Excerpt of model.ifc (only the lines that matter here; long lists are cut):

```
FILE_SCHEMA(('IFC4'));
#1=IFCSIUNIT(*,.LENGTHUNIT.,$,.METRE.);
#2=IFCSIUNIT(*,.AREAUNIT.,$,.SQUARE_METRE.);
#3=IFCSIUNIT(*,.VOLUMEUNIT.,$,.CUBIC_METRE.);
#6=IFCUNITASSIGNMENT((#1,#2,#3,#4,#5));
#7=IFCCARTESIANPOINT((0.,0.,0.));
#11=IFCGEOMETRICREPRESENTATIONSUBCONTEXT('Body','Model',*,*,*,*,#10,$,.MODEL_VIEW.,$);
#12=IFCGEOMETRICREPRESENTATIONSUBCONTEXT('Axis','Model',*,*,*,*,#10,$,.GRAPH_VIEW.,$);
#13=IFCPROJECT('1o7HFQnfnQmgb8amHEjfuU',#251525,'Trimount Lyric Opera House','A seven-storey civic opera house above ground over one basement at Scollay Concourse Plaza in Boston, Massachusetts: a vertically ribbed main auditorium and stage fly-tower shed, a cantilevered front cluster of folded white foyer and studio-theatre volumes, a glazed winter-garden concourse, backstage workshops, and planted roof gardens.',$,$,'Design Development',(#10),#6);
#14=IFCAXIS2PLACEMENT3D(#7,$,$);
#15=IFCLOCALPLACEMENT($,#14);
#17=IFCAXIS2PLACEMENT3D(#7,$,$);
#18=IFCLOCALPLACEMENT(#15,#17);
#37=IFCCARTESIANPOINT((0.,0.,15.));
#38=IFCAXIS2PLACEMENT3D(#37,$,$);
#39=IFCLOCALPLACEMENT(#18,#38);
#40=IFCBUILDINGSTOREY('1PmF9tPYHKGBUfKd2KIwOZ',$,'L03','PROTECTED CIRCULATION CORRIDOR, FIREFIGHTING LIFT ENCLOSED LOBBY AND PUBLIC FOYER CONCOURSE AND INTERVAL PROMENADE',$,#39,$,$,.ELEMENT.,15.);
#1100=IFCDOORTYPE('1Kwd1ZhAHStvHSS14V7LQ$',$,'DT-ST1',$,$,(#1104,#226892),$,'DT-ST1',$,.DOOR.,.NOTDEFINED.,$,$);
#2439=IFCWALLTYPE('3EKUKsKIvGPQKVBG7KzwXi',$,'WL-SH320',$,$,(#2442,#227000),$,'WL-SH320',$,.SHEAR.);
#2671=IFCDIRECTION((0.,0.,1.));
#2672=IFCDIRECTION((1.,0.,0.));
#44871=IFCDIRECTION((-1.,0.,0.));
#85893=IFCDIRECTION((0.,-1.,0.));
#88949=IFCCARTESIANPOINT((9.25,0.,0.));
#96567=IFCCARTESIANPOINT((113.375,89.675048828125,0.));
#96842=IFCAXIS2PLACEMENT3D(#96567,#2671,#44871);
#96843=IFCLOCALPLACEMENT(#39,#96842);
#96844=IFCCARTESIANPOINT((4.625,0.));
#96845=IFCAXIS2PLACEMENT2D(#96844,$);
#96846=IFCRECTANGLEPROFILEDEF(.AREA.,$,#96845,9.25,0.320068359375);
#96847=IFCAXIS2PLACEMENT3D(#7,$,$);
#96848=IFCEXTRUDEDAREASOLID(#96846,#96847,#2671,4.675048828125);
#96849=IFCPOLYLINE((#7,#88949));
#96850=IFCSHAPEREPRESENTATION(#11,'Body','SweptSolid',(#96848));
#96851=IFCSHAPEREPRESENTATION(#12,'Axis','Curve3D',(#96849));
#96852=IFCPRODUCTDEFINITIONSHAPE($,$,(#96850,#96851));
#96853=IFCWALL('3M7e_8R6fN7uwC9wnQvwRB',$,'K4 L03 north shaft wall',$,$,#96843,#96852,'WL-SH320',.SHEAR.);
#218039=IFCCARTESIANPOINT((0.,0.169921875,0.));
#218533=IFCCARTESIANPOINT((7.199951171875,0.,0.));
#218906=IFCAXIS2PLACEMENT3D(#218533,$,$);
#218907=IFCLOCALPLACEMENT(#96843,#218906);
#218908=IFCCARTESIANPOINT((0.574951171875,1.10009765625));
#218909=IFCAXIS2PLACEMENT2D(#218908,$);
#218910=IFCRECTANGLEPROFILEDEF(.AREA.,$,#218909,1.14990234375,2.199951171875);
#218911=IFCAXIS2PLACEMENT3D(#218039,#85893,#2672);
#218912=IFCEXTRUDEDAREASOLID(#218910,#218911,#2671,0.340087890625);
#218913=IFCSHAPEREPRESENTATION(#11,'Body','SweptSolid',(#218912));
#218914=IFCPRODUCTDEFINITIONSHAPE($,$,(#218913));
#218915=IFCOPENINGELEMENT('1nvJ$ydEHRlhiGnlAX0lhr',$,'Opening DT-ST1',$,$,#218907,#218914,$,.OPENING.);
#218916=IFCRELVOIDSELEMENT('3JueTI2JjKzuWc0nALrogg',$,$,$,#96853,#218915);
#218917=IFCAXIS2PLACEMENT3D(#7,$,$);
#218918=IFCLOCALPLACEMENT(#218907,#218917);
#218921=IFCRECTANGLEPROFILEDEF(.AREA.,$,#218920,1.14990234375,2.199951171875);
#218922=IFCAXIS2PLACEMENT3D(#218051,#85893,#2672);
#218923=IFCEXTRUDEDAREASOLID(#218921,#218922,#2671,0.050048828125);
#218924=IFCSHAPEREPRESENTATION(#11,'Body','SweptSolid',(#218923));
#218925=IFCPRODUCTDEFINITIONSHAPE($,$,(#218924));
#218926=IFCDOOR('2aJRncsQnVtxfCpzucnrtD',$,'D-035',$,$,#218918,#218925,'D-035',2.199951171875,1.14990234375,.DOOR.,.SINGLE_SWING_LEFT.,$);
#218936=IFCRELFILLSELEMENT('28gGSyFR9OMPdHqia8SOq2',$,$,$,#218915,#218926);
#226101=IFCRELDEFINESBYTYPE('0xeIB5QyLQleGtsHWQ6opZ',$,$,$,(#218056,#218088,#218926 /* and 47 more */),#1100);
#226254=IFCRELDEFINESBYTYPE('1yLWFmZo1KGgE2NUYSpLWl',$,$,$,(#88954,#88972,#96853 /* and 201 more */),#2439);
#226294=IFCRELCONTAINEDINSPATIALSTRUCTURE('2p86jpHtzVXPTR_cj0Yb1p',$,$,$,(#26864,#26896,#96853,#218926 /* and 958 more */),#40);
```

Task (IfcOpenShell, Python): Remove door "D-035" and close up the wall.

```python
import ifcopenshell
import ifcopenshell.api.feature
import ifcopenshell.api.root
import ifcopenshell.geom
import ifcopenshell.util.shape

model = ifcopenshell.open("model.ifc")
settings = ifcopenshell.geom.settings()


def volume(element):
    """Net volume in cubic metres, openings subtracted."""
    shape = ifcopenshell.geom.create_shape(settings, element)
    return ifcopenshell.util.shape.get_volume(shape.geometry)


door = model.by_guid("2aJRncsQnVtxfCpzucnrtD")
opening = door.FillsVoids[0].RelatingOpeningElement
wall = opening.VoidsElements[0].RelatingBuildingElement
before = volume(wall)

ifcopenshell.api.root.remove_product(model, product=door)
ifcopenshell.api.feature.remove_feature(model, feature=opening)

after = volume(wall)

print(f"wall volume {before:.3f} -> {after:.3f} m3")

model.write("model_edited.ifc")
```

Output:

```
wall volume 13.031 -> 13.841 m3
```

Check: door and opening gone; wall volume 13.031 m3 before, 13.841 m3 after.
